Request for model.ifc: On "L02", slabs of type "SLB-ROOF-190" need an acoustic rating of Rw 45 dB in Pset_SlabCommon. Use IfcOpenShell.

First a look at what the model holds.

```python
import ifcopenshell
import ifcopenshell.util.element

model = ifcopenshell.open("model.ifc")
print(model.schema)
storey = next(s for s in model.by_type("IfcBuildingStorey") if s.Name == "L02")
slabs = [e for e in ifcopenshell.util.element.get_decomposition(storey) if e.is_a("IfcSlab")]
seen = {}
for e in slabs:
    element_type = ifcopenshell.util.element.get_type(e)
    key = (element_type.Name if element_type != e and element_type else None, ifcopenshell.util.element.get_pset(e, "Pset_SlabCommon", "AcousticRating"))
    seen[key] = seen.get(key, 0) + 1
for (name, value), count in sorted(seen.items(), key=str):
    print(count, "x", name, "|", value)
```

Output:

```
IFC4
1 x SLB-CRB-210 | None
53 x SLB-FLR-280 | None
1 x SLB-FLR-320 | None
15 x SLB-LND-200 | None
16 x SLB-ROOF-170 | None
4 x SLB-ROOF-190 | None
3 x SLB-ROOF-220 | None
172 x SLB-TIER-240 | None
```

```python
import ifcopenshell
import ifcopenshell.api.pset
import ifcopenshell.util.element

model = ifcopenshell.open("model.ifc")

storey = next(s for s in model.by_type("IfcBuildingStorey") if s.Name == "L02")
slabs = [e for e in ifcopenshell.util.element.get_decomposition(storey) if e.is_a("IfcSlab")]

count = 0
for e in slabs:
    element_type = ifcopenshell.util.element.get_type(e)
    if element_type in (None, e) or element_type.Name != "SLB-ROOF-190":
        continue
    # add_pset returns the element's existing set when there is one.
    pset = ifcopenshell.api.pset.add_pset(model, product=e, name="Pset_SlabCommon")
    ifcopenshell.api.pset.edit_pset(model, pset=pset, properties={"AcousticRating": "Rw 45 dB"})
    count += 1

print(count, "slabs updated")

model.write("model_edited.ifc")
```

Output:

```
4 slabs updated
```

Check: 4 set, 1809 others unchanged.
